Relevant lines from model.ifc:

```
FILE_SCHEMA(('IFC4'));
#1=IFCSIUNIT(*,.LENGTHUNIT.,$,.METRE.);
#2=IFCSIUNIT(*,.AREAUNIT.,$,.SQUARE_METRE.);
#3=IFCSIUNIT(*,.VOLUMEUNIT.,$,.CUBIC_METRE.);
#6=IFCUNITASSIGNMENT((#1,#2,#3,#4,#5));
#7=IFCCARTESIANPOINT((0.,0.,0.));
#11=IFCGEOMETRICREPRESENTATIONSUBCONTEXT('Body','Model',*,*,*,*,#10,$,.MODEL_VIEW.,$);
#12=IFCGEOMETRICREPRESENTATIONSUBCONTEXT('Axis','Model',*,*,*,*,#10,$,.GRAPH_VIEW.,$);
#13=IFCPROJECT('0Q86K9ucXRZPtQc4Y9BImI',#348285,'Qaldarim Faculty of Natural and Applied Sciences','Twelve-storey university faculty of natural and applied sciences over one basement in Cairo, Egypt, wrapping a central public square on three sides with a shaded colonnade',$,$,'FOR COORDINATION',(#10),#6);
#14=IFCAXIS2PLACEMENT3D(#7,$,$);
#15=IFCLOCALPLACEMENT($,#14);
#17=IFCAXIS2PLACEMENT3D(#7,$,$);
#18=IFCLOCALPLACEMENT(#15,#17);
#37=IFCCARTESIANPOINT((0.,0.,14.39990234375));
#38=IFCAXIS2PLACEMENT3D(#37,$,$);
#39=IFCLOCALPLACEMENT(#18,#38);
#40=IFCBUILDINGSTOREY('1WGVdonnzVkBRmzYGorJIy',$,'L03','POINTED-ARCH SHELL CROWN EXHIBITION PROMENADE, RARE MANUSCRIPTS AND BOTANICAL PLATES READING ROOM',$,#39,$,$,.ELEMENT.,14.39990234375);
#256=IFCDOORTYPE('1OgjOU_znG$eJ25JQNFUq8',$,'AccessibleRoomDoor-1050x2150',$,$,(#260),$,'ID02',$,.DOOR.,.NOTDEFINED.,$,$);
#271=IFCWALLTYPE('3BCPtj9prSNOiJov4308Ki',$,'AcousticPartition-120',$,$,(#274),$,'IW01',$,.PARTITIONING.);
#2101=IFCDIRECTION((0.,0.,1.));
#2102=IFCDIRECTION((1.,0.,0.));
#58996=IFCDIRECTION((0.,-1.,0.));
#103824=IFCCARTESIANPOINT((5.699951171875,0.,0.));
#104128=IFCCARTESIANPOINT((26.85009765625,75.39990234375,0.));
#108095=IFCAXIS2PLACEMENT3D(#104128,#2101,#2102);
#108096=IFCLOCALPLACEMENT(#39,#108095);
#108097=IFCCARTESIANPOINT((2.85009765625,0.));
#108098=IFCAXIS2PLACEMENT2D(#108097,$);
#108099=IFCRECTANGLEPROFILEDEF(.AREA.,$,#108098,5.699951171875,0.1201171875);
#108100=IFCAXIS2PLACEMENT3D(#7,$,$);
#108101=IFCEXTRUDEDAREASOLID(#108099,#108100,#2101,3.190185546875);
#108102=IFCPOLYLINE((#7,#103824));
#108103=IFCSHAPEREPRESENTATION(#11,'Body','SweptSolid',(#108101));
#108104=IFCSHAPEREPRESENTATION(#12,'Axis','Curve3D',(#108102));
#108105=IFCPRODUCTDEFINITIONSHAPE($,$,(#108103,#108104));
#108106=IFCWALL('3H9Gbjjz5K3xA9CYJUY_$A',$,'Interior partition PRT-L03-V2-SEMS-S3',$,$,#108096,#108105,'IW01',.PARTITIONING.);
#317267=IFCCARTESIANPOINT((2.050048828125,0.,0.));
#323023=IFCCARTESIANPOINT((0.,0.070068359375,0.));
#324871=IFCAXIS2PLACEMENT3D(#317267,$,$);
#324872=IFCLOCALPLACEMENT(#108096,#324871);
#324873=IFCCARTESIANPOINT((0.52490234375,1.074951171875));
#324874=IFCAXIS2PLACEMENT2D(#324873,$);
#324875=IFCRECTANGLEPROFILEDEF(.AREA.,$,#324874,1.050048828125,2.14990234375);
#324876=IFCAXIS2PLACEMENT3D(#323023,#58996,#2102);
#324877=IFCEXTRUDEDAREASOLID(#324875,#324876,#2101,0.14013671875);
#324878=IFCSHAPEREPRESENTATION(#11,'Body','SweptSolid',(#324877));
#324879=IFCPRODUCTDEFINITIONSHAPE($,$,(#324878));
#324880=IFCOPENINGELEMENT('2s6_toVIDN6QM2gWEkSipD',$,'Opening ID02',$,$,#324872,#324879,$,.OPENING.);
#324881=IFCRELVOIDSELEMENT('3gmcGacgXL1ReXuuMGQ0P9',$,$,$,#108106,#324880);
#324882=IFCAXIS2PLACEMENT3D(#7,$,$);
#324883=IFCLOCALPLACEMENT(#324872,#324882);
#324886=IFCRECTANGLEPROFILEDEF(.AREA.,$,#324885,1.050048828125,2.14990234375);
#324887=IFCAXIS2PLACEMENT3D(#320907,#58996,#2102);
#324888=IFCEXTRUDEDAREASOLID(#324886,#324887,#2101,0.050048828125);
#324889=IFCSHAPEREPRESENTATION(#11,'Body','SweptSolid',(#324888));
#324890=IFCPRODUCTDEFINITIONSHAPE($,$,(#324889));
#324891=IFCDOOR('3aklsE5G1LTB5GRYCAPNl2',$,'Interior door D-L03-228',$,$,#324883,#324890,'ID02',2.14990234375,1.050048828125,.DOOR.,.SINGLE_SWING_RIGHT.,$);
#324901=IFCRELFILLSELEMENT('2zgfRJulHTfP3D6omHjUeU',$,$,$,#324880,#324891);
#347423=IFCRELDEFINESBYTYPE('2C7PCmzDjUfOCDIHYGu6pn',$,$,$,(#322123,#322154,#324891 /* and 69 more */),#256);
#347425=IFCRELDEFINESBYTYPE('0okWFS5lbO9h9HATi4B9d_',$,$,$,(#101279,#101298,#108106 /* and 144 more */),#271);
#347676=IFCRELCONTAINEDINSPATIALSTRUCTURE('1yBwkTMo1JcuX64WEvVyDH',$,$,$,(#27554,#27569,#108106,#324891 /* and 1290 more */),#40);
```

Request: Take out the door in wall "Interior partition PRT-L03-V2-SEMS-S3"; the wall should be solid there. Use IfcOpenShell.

```python
import ifcopenshell
import ifcopenshell.api.feature
import ifcopenshell.api.root
import ifcopenshell.geom
import ifcopenshell.util.shape

model = ifcopenshell.open("model.ifc")
settings = ifcopenshell.geom.settings()


def volume(element):
    """Net volume in cubic metres, openings subtracted."""
    shape = ifcopenshell.geom.create_shape(settings, element)
    return ifcopenshell.util.shape.get_volume(shape.geometry)


door = model.by_guid("3aklsE5G1LTB5GRYCAPNl2")
opening = door.FillsVoids[0].RelatingOpeningElement
wall = opening.VoidsElements[0].RelatingBuildingElement
before = volume(wall)

ifcopenshell.api.root.remove_product(model, product=door)
ifcopenshell.api.feature.remove_feature(model, feature=opening)

after = volume(wall)

print(f"wall volume {before:.3f} -> {after:.3f} m3")

model.write("model-out.ifc")
```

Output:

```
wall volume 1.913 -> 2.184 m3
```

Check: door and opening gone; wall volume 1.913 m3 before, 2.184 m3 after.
